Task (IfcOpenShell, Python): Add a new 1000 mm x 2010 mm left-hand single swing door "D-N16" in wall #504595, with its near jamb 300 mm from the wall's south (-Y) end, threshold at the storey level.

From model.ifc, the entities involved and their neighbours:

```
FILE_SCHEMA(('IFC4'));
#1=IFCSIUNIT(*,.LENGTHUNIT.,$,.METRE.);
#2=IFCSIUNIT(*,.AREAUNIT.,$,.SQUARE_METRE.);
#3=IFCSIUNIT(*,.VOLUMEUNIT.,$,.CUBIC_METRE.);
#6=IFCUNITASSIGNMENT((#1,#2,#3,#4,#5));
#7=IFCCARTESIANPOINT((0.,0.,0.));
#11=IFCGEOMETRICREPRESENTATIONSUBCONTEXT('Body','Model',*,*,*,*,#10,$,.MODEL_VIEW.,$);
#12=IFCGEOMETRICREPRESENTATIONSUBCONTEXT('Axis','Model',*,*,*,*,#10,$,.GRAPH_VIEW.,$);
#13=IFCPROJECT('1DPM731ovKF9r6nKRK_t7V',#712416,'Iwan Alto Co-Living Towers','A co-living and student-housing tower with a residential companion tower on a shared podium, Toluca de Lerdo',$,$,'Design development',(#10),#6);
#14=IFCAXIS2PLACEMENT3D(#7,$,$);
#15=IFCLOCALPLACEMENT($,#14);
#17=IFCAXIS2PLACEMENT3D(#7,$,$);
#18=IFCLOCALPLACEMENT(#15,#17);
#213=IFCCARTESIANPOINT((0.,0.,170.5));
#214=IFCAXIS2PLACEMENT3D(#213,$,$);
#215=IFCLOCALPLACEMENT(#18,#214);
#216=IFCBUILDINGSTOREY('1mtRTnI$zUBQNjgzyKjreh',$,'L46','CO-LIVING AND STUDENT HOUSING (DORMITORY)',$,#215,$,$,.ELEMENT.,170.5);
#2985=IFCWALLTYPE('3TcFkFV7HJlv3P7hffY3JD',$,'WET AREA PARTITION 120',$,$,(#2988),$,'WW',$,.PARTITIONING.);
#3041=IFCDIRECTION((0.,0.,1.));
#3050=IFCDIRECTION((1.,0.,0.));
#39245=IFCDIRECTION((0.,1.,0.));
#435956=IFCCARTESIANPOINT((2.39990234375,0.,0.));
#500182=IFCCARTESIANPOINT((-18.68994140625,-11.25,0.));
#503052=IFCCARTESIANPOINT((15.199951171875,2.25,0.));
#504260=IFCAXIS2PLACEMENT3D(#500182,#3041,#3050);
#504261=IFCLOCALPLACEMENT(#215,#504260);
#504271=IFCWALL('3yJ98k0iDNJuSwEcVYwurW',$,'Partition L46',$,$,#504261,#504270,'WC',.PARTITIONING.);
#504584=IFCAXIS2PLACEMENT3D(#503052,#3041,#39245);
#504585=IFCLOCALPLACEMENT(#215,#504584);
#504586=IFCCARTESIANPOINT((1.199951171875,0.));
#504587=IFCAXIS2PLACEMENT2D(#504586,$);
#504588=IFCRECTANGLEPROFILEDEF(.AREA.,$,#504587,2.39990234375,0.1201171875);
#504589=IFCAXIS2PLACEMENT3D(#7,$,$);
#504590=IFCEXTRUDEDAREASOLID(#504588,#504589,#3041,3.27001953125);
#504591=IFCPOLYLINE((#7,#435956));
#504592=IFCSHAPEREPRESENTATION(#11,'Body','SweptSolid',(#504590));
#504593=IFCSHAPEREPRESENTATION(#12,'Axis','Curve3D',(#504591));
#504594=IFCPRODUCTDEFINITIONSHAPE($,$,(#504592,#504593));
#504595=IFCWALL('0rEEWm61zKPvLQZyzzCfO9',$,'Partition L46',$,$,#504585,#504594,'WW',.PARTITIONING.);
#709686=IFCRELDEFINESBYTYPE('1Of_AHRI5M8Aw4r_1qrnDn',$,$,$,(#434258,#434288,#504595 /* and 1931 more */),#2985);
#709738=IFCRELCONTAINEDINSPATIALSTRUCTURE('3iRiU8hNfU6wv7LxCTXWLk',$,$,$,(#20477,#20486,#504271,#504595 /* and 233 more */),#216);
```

```python
import numpy as np
import ifcopenshell
import ifcopenshell.api.feature
import ifcopenshell.api.geometry
import ifcopenshell.api.root
import ifcopenshell.api.spatial
import ifcopenshell.geom
import ifcopenshell.util.element
import ifcopenshell.util.placement
import ifcopenshell.util.representation
import ifcopenshell.util.shape
import ifcopenshell.util.unit

model = ifcopenshell.open("model.ifc")
unit_scale = ifcopenshell.util.unit.calculate_unit_scale(model)
settings = ifcopenshell.geom.settings()


def volume(element):
    """Net volume in cubic metres, openings subtracted."""
    shape = ifcopenshell.geom.create_shape(settings, element)
    return ifcopenshell.util.shape.get_volume(shape.geometry)


wall = model.by_guid("0rEEWm61zKPvLQZyzzCfO9")
storey = ifcopenshell.util.element.get_container(wall, ifc_class="IfcBuildingStorey")
context = ifcopenshell.util.representation.get_context(model, "Model", "Body", "MODEL_VIEW")
before = volume(wall)

width, height, from_end, sill = 1, 2.01, 0.3, 0.0  # metres

# The wall runs along its own X axis, and the end named is its -X end.
wall_shape = ifcopenshell.geom.create_shape(settings, wall)
x, y, z = ifcopenshell.util.shape.get_vertices(wall_shape.geometry).T
start = x.min() + from_end
face, thickness = float(y.min()), float(y.max() - y.min())
wall_matrix = ifcopenshell.util.placement.get_local_placement(wall.ObjectPlacement)
level = ifcopenshell.util.placement.get_local_placement(storey.ObjectPlacement)[2, 3]


def in_wall(x, y):
    """Placement at x, y metres in the wall's axes, at sill height."""
    matrix = wall_matrix.copy()
    matrix[:, 3] = wall_matrix @ np.array([x / unit_scale, y / unit_scale, 0.0, 1.0])
    matrix[2, 3] = level + sill / unit_scale
    return matrix


# Opening: a box that overshoots both wall faces by 50 mm.
opening = ifcopenshell.api.root.create_entity(model, ifc_class="IfcOpeningElement", predefined_type="OPENING")
box = ifcopenshell.api.geometry.add_wall_representation(
    model, context=context, length=width, height=height, thickness=thickness + 0.1
)
ifcopenshell.api.geometry.assign_representation(model, product=opening, representation=box)
ifcopenshell.api.geometry.edit_object_placement(model, product=opening, matrix=in_wall(start, face - 0.05), is_si=False)
ifcopenshell.api.feature.add_feature(model, feature=opening, element=wall)

door = ifcopenshell.api.root.create_entity(model, ifc_class="IfcDoor", name="D-N16", predefined_type="DOOR")
door.OverallWidth, door.OverallHeight = width / unit_scale, height / unit_scale
door.OperationType = "SINGLE_SWING_LEFT"
body = ifcopenshell.api.geometry.add_door_representation(
    model,
    context=context,
    overall_width=door.OverallWidth,
    overall_height=door.OverallHeight,
    operation_type="SINGLE_SWING_LEFT",
    lining_properties={"LiningDepth": thickness / unit_scale, "ThresholdDepth": thickness / unit_scale},
)
ifcopenshell.api.geometry.assign_representation(model, product=door, representation=body)
ifcopenshell.api.spatial.assign_container(model, products=[door], relating_structure=storey)
ifcopenshell.api.feature.add_filling(model, opening=opening, element=door)

# The lining spans the wall, so the door starts at the wall face.
ifcopenshell.api.geometry.edit_object_placement(model, product=door, matrix=in_wall(start, face), is_si=False)

after = volume(wall)

print(f"wall volume {before:.3f} -> {after:.3f} m3")

model.write("model_v2.ifc")
```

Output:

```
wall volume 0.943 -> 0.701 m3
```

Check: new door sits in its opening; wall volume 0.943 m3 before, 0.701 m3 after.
